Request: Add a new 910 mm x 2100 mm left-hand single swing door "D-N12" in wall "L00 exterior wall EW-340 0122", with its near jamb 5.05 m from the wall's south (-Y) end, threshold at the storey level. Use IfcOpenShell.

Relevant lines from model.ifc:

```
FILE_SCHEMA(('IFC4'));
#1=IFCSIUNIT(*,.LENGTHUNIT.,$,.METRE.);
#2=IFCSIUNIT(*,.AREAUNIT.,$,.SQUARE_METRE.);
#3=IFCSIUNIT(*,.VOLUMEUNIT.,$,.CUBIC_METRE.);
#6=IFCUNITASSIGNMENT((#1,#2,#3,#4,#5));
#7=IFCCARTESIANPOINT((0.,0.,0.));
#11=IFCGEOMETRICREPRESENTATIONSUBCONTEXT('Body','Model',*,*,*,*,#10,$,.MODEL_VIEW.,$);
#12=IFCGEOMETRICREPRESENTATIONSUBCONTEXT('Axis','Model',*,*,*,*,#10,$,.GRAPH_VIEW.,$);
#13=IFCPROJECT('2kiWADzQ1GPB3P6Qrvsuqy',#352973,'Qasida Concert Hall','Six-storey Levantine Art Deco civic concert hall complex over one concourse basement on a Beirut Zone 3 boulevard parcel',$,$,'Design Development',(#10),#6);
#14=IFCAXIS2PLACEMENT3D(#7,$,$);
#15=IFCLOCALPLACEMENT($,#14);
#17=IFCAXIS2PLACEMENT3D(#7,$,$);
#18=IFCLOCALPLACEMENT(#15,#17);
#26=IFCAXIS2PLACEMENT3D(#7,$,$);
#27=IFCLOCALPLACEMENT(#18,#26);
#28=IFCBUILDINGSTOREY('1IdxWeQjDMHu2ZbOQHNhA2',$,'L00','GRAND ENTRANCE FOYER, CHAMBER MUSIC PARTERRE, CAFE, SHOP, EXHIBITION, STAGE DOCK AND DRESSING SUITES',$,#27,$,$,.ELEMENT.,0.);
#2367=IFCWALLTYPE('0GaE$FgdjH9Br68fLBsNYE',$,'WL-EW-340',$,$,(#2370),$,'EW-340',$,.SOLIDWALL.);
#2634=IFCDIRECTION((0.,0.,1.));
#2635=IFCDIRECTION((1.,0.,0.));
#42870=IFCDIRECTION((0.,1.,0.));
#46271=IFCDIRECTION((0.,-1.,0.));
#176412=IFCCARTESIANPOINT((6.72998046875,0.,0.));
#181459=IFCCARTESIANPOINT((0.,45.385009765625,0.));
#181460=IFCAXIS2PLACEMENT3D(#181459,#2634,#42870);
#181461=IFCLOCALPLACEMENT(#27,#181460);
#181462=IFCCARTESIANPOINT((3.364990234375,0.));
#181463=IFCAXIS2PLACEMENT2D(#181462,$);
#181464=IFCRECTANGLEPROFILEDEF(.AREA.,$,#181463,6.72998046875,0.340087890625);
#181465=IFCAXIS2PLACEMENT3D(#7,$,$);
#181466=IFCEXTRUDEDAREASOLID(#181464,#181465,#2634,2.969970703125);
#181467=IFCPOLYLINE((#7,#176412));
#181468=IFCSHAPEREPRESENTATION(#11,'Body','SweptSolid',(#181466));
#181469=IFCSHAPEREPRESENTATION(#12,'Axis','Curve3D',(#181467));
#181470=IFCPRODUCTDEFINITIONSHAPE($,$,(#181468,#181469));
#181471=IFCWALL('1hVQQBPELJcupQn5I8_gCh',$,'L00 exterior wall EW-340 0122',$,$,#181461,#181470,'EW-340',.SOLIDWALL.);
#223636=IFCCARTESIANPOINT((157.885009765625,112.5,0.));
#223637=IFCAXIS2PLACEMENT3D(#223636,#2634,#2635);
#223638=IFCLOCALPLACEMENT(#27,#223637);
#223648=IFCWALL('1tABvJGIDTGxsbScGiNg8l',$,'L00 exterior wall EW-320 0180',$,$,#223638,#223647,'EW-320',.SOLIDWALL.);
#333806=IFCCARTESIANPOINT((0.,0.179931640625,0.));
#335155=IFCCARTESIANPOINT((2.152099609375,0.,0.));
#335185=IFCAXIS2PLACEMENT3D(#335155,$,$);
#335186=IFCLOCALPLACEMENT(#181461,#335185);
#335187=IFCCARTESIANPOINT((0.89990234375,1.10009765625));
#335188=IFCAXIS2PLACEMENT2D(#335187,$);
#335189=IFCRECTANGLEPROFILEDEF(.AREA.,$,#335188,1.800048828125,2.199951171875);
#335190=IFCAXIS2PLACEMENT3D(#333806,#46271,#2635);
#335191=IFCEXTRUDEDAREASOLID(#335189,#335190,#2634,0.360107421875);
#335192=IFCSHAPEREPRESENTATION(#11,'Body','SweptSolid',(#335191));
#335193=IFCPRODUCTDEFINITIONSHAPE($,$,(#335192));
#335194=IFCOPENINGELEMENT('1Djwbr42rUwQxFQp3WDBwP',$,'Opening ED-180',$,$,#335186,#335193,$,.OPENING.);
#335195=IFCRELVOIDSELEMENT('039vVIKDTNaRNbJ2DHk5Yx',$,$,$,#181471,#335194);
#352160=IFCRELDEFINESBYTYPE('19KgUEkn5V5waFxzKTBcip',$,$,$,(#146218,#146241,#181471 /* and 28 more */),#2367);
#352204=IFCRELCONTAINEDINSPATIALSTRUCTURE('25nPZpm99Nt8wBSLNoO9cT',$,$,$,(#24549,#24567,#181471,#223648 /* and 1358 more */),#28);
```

```python
import numpy as np
import ifcopenshell
import ifcopenshell.api.feature
import ifcopenshell.api.geometry
import ifcopenshell.api.root
import ifcopenshell.api.spatial
import ifcopenshell.geom
import ifcopenshell.util.element
import ifcopenshell.util.placement
import ifcopenshell.util.representation
import ifcopenshell.util.shape
import ifcopenshell.util.unit

model = ifcopenshell.open("model.ifc")
unit_scale = ifcopenshell.util.unit.calculate_unit_scale(model)
settings = ifcopenshell.geom.settings()


def volume(element):
    """Net volume in cubic metres, openings subtracted."""
    shape = ifcopenshell.geom.create_shape(settings, element)
    return ifcopenshell.util.shape.get_volume(shape.geometry)


wall = model.by_id(181471)
storey = ifcopenshell.util.element.get_container(wall, ifc_class="IfcBuildingStorey")
context = ifcopenshell.util.representation.get_context(model, "Model", "Body", "MODEL_VIEW")
before = volume(wall)

width, height, from_end, sill = 0.91, 2.1, 5.05, 0.0  # metres

# The wall runs along its own X axis, and the end named is its -X end.
wall_shape = ifcopenshell.geom.create_shape(settings, wall)
x, y, z = ifcopenshell.util.shape.get_vertices(wall_shape.geometry).T
start = x.min() + from_end
face, thickness = float(y.min()), float(y.max() - y.min())
wall_matrix = ifcopenshell.util.placement.get_local_placement(wall.ObjectPlacement)
level = ifcopenshell.util.placement.get_local_placement(storey.ObjectPlacement)[2, 3]


def in_wall(x, y):
    """Placement at x, y metres in the wall's axes, at sill height."""
    matrix = wall_matrix.copy()
    matrix[:, 3] = wall_matrix @ np.array([x / unit_scale, y / unit_scale, 0.0, 1.0])
    matrix[2, 3] = level + sill / unit_scale
    return matrix


# Opening: a box that overshoots both wall faces by 50 mm.
opening = ifcopenshell.api.root.create_entity(model, ifc_class="IfcOpeningElement", predefined_type="OPENING")
box = ifcopenshell.api.geometry.add_wall_representation(
    model, context=context, length=width, height=height, thickness=thickness + 0.1
)
ifcopenshell.api.geometry.assign_representation(model, product=opening, representation=box)
ifcopenshell.api.geometry.edit_object_placement(model, product=opening, matrix=in_wall(start, face - 0.05), is_si=False)
ifcopenshell.api.feature.add_feature(model, feature=opening, element=wall)

door = ifcopenshell.api.root.create_entity(model, ifc_class="IfcDoor", name="D-N12", predefined_type="DOOR")
door.OverallWidth, door.OverallHeight = width / unit_scale, height / unit_scale
door.OperationType = "SINGLE_SWING_LEFT"
body = ifcopenshell.api.geometry.add_door_representation(
    model,
    context=context,
    overall_width=door.OverallWidth,
    overall_height=door.OverallHeight,
    operation_type="SINGLE_SWING_LEFT",
    lining_properties={"LiningDepth": thickness / unit_scale, "ThresholdDepth": thickness / unit_scale},
)
ifcopenshell.api.geometry.assign_representation(model, product=door, representation=body)
ifcopenshell.api.spatial.assign_container(model, products=[door], relating_structure=storey)
ifcopenshell.api.feature.add_filling(model, opening=opening, element=door)

# The lining spans the wall, so the door starts at the wall face.
ifcopenshell.api.geometry.edit_object_placement(model, product=door, matrix=in_wall(start, face), is_si=False)

after = volume(wall)

print(f"wall volume {before:.3f} -> {after:.3f} m3")

model.write("model_rev.ifc")
```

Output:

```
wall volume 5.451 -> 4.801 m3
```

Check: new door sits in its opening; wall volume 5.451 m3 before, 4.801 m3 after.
